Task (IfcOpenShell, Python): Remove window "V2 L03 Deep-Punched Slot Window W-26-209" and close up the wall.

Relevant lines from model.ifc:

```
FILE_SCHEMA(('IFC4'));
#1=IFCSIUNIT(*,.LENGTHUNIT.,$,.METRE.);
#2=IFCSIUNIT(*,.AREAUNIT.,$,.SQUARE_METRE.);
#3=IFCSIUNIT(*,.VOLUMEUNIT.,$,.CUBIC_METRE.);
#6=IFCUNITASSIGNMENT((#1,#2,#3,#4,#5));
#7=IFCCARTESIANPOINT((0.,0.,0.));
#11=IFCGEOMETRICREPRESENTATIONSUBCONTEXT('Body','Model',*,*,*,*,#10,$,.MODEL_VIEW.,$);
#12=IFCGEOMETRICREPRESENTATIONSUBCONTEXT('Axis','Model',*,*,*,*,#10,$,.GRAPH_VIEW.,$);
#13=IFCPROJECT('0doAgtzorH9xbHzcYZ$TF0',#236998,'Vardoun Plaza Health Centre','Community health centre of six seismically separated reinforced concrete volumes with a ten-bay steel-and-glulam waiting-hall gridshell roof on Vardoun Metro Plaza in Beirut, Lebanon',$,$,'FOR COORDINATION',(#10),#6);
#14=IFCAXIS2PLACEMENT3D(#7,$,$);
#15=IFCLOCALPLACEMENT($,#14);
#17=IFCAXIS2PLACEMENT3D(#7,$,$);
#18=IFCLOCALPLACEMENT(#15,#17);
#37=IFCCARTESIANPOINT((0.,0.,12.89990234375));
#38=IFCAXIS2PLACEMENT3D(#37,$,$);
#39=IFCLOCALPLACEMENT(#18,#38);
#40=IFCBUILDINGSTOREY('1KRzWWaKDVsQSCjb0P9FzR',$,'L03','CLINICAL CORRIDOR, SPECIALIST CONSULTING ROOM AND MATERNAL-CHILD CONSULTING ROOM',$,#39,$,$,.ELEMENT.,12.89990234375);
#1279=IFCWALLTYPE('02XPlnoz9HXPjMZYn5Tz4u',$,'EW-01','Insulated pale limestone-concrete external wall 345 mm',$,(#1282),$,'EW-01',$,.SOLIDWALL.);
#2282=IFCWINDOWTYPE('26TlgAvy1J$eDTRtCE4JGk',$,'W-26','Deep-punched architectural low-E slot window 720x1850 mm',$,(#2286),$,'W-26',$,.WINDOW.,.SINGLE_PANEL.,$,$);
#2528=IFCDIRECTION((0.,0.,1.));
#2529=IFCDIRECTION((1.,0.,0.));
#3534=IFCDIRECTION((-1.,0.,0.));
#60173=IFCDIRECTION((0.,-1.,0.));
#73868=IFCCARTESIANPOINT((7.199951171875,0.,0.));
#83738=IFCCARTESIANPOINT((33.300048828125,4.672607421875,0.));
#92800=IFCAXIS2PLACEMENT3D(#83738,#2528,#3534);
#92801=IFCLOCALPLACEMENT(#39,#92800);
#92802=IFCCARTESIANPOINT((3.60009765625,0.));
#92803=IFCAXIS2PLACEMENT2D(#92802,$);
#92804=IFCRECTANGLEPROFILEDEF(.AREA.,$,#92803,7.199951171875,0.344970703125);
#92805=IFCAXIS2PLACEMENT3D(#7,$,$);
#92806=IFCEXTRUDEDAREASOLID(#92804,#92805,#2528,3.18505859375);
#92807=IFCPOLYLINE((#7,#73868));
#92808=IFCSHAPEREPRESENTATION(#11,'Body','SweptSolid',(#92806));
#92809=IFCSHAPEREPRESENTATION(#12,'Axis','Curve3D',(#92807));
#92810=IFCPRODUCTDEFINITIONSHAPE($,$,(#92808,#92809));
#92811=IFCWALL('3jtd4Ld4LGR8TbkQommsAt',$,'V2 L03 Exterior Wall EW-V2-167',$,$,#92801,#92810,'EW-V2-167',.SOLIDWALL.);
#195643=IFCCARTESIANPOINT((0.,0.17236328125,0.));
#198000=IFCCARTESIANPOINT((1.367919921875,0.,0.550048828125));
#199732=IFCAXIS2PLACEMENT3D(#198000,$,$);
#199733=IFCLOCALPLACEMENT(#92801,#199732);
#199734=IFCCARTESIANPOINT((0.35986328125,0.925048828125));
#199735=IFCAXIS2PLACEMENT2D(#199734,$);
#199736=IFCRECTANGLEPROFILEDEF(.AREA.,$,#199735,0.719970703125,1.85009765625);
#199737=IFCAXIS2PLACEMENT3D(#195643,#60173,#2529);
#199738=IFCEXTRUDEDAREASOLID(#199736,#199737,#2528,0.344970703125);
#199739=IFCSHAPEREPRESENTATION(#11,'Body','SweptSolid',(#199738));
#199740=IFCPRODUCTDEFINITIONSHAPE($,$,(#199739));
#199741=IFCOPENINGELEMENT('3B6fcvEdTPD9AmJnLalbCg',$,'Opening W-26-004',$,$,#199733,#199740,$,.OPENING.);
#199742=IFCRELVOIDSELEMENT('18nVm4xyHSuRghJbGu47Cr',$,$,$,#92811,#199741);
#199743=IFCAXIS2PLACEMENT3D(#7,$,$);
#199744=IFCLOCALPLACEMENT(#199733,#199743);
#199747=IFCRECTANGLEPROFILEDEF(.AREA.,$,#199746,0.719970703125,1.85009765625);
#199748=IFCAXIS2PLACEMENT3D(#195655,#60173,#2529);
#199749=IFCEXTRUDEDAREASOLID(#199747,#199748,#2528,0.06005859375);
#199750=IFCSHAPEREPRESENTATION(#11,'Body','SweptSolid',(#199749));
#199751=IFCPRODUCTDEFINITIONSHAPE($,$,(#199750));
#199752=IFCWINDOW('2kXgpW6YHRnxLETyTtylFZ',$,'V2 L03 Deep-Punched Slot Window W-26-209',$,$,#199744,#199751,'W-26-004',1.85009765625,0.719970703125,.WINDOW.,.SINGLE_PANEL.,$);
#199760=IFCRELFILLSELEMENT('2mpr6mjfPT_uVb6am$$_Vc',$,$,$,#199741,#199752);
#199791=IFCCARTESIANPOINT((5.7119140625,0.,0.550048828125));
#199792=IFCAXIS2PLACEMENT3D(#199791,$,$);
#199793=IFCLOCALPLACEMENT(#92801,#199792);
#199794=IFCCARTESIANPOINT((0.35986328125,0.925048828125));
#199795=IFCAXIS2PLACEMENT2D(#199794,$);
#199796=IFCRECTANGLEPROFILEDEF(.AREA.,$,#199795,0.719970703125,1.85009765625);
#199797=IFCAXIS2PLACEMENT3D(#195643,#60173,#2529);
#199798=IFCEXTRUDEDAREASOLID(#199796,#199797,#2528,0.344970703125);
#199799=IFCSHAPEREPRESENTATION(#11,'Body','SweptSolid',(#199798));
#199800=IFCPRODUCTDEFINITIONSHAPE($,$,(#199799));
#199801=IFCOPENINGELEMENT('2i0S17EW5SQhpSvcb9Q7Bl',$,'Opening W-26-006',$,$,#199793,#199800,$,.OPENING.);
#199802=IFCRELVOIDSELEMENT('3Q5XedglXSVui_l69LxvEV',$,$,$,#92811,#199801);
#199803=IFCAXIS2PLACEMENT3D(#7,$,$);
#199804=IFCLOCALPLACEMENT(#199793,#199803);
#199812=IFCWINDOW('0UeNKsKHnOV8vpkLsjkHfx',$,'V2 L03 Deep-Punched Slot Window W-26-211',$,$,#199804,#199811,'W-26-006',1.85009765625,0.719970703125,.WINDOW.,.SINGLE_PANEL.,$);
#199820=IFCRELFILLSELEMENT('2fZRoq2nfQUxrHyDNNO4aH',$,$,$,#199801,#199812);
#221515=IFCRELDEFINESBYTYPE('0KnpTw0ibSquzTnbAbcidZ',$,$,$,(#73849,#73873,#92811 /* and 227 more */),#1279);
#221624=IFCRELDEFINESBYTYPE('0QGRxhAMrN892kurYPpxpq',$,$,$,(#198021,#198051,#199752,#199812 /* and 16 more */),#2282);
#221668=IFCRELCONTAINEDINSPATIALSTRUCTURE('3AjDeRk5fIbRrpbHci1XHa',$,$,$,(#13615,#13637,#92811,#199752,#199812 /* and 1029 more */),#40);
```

```python
import ifcopenshell
import ifcopenshell.api.feature
import ifcopenshell.api.root
import ifcopenshell.geom
import ifcopenshell.util.shape

model = ifcopenshell.open("model.ifc")
settings = ifcopenshell.geom.settings()


def volume(element):
    """Net volume in cubic metres, openings subtracted."""
    shape = ifcopenshell.geom.create_shape(settings, element)
    return ifcopenshell.util.shape.get_volume(shape.geometry)


window = model.by_id(199752)
opening = window.FillsVoids[0].RelatingOpeningElement
wall = opening.VoidsElements[0].RelatingBuildingElement
before = volume(wall)

ifcopenshell.api.root.remove_product(model, product=window)
ifcopenshell.api.feature.remove_feature(model, feature=opening)

after = volume(wall)

print(f"wall volume {before:.3f} -> {after:.3f} m3")

model.write("model_updated.ifc")
```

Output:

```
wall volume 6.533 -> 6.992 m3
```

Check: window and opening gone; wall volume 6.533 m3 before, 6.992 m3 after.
